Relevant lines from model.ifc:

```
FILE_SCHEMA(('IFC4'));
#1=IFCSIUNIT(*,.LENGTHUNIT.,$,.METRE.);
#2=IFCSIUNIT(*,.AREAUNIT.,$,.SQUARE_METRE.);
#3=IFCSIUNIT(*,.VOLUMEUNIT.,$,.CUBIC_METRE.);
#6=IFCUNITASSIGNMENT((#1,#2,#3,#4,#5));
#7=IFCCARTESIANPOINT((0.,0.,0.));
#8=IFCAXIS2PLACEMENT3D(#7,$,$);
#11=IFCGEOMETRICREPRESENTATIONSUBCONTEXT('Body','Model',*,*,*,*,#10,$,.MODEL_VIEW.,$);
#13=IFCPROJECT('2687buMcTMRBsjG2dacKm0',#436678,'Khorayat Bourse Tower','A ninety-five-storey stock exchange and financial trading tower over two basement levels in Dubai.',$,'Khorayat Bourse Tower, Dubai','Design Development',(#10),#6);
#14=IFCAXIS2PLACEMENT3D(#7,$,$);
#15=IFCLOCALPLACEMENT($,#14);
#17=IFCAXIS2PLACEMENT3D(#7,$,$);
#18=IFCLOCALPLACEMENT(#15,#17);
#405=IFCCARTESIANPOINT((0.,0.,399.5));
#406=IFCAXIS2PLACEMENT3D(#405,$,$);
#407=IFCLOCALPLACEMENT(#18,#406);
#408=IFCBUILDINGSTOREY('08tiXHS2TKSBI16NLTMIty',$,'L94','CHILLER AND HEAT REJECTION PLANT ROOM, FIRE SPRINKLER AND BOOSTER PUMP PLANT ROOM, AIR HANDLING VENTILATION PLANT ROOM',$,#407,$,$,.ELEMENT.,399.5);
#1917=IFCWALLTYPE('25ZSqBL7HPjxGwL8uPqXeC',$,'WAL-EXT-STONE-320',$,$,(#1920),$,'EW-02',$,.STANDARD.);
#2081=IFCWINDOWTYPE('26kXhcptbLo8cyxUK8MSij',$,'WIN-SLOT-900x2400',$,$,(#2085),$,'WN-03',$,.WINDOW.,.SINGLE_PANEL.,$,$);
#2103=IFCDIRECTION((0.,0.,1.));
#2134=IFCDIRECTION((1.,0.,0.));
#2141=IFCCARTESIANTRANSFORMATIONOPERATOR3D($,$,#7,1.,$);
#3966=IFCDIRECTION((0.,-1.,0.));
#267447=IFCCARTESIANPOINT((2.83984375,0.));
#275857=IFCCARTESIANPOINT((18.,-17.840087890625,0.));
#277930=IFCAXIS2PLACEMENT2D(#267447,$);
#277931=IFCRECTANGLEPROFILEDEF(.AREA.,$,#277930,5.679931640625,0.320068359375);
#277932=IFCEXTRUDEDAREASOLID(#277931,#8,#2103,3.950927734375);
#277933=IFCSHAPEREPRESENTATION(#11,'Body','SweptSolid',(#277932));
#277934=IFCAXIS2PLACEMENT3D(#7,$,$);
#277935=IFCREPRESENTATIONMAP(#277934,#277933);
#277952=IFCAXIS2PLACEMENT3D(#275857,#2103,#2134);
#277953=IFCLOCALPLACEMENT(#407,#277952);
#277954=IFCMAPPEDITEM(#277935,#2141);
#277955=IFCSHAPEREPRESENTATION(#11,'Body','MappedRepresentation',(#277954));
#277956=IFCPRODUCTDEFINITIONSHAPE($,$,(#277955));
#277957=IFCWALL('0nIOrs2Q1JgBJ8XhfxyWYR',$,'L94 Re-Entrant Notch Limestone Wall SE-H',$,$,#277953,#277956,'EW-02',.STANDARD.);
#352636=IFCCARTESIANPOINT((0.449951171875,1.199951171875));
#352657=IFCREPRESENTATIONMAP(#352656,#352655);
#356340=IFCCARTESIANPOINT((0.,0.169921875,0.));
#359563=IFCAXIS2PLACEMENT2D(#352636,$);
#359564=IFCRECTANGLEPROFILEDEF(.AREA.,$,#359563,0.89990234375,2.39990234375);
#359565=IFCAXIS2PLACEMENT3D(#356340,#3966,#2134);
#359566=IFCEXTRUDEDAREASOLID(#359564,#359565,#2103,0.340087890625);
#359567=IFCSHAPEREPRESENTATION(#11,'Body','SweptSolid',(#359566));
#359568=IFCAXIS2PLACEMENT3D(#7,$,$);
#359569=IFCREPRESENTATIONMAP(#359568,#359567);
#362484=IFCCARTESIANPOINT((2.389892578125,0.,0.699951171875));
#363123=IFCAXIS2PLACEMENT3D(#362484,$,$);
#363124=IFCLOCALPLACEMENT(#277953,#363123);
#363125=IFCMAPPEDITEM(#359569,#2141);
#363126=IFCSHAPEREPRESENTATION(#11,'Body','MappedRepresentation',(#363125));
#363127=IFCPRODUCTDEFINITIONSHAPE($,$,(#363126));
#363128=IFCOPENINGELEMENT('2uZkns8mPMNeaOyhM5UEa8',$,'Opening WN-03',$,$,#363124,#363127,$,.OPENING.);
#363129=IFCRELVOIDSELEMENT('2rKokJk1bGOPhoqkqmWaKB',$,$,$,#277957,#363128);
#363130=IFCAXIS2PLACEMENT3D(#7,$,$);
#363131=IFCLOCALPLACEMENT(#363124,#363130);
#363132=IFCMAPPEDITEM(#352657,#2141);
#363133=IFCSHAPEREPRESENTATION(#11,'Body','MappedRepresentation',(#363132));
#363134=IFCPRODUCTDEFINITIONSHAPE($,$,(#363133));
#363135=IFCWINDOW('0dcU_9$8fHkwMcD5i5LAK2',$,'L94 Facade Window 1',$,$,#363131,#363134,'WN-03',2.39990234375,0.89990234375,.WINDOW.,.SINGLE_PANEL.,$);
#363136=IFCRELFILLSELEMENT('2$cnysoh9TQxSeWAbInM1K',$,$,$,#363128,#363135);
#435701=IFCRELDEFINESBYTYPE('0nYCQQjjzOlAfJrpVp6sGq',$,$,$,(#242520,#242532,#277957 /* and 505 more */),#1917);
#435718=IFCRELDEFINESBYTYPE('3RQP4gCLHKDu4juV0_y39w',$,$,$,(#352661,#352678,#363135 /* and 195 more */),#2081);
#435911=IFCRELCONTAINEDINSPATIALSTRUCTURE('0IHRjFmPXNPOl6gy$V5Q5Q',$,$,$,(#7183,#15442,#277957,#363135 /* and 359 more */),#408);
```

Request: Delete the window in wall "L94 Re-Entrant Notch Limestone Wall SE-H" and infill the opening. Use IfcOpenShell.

```python
import ifcopenshell
import ifcopenshell.api.feature
import ifcopenshell.api.root
import ifcopenshell.geom
import ifcopenshell.util.shape

model = ifcopenshell.open("model.ifc")
settings = ifcopenshell.geom.settings()


def volume(element):
    """Net volume in cubic metres, openings subtracted."""
    shape = ifcopenshell.geom.create_shape(settings, element)
    return ifcopenshell.util.shape.get_volume(shape.geometry)


window = model.by_guid("0dcU_9$8fHkwMcD5i5LAK2")
opening = window.FillsVoids[0].RelatingOpeningElement
wall = opening.VoidsElements[0].RelatingBuildingElement
before = volume(wall)

ifcopenshell.api.root.remove_product(model, product=window)
ifcopenshell.api.feature.remove_feature(model, feature=opening)

after = volume(wall)

print(f"wall volume {before:.3f} -> {after:.3f} m3")

model.write("model_rev.ifc")
```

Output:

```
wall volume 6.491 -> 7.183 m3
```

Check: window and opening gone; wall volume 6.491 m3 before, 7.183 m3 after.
